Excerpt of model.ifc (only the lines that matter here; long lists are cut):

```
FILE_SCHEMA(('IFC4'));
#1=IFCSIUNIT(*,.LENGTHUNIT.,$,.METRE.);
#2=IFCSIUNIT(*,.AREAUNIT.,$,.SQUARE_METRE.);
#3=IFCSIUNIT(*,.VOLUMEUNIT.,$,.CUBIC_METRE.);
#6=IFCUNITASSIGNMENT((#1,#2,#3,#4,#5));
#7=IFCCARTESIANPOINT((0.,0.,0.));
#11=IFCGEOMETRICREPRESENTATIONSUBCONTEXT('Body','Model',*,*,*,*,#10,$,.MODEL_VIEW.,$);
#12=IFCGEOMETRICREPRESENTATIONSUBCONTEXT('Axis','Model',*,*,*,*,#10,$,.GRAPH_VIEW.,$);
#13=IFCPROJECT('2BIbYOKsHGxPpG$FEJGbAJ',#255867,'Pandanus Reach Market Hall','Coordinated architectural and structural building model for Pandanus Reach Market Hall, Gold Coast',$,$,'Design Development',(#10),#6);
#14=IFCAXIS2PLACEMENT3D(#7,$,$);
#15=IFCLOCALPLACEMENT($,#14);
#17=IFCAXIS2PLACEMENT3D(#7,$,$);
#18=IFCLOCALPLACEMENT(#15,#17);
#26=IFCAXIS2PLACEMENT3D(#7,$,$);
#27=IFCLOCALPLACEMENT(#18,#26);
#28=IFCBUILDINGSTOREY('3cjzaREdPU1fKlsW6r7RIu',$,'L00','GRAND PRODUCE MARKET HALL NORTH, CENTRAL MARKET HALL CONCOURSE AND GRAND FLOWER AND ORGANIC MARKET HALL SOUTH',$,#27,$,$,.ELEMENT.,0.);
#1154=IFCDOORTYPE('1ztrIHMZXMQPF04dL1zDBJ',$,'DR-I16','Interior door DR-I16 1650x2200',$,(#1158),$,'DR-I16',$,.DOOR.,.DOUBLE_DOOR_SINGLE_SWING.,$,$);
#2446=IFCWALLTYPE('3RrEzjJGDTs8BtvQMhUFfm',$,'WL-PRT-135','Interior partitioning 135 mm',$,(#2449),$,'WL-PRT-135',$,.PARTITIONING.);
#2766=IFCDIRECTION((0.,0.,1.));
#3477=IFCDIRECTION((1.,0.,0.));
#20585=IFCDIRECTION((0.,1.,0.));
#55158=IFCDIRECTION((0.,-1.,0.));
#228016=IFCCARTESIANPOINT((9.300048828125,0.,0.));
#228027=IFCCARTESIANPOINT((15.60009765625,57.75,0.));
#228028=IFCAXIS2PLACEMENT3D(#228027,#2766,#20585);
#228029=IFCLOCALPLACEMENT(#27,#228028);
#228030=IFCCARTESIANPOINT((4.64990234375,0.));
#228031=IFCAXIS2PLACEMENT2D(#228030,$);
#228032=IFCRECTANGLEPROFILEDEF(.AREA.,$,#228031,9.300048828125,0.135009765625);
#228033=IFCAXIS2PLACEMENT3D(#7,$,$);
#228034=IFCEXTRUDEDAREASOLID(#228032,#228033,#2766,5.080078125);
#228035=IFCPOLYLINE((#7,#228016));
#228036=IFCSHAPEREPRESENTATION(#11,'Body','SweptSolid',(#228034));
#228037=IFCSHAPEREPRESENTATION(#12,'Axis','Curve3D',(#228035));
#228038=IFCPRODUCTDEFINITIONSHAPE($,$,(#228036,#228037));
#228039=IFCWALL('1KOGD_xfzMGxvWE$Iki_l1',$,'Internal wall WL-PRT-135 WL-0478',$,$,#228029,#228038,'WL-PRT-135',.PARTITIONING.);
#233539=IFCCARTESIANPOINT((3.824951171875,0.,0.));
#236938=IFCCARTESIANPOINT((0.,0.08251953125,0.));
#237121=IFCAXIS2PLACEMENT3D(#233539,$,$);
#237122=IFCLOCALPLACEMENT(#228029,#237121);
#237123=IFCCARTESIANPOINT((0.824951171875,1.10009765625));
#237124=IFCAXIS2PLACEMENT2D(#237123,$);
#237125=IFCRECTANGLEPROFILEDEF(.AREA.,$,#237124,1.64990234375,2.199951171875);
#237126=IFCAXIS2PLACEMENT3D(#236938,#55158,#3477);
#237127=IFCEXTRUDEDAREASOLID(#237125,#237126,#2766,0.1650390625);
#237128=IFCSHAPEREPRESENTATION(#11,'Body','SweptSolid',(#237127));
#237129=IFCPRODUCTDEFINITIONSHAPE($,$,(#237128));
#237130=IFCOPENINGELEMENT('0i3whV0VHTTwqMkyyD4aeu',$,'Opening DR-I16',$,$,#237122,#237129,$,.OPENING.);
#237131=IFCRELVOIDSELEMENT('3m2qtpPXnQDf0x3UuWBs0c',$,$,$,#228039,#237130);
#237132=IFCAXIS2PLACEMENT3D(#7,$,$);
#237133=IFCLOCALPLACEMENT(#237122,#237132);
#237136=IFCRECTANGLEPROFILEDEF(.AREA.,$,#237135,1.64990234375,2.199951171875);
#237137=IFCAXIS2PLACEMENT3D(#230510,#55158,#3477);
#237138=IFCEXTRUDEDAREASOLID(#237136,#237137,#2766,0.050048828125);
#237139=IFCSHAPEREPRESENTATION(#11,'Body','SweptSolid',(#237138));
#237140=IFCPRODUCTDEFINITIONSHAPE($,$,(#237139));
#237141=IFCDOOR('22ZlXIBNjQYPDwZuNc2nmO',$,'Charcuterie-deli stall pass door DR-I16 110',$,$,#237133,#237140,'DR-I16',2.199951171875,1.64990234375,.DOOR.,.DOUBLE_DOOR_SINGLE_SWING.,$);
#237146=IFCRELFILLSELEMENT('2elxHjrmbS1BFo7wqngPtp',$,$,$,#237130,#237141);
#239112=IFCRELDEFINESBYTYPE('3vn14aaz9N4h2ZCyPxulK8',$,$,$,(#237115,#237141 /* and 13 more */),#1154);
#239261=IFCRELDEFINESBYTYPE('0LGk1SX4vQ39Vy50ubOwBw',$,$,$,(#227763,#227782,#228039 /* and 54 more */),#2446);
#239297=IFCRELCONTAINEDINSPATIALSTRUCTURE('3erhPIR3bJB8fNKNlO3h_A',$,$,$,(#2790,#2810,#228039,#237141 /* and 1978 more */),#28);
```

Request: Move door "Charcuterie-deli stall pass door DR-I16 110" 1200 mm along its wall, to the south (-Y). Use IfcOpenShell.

```python
import ifcopenshell
import ifcopenshell.api.geometry
import ifcopenshell.util.placement
import ifcopenshell.util.unit

model = ifcopenshell.open("model.ifc")
unit_scale = ifcopenshell.util.unit.calculate_unit_scale(model)

door = model.by_guid("22ZlXIBNjQYPDwZuNc2nmO")
opening = door.FillsVoids[0].RelatingOpeningElement
wall = opening.VoidsElements[0].RelatingBuildingElement

wall_matrix = ifcopenshell.util.placement.get_local_placement(wall.ObjectPlacement)
shift = wall_matrix[:3, 0] * -1.2 / unit_scale
before = ifcopenshell.util.placement.get_local_placement(door.ObjectPlacement)[:3, 3].copy()

# The door is placed relative to its opening, so it follows when the opening moves.
matrix = ifcopenshell.util.placement.get_local_placement(opening.ObjectPlacement)
matrix[:3, 3] += shift
ifcopenshell.api.geometry.edit_object_placement(
    model, product=opening, matrix=matrix, is_si=False, should_transform_children=True
)

after = ifcopenshell.util.placement.get_local_placement(door.ObjectPlacement)[:3, 3]
print("door moved by", (after - before).round(3) + 0.0)

model.write("model_edited.ifc")
```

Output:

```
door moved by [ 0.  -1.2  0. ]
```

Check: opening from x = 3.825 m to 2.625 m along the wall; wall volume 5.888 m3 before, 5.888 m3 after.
